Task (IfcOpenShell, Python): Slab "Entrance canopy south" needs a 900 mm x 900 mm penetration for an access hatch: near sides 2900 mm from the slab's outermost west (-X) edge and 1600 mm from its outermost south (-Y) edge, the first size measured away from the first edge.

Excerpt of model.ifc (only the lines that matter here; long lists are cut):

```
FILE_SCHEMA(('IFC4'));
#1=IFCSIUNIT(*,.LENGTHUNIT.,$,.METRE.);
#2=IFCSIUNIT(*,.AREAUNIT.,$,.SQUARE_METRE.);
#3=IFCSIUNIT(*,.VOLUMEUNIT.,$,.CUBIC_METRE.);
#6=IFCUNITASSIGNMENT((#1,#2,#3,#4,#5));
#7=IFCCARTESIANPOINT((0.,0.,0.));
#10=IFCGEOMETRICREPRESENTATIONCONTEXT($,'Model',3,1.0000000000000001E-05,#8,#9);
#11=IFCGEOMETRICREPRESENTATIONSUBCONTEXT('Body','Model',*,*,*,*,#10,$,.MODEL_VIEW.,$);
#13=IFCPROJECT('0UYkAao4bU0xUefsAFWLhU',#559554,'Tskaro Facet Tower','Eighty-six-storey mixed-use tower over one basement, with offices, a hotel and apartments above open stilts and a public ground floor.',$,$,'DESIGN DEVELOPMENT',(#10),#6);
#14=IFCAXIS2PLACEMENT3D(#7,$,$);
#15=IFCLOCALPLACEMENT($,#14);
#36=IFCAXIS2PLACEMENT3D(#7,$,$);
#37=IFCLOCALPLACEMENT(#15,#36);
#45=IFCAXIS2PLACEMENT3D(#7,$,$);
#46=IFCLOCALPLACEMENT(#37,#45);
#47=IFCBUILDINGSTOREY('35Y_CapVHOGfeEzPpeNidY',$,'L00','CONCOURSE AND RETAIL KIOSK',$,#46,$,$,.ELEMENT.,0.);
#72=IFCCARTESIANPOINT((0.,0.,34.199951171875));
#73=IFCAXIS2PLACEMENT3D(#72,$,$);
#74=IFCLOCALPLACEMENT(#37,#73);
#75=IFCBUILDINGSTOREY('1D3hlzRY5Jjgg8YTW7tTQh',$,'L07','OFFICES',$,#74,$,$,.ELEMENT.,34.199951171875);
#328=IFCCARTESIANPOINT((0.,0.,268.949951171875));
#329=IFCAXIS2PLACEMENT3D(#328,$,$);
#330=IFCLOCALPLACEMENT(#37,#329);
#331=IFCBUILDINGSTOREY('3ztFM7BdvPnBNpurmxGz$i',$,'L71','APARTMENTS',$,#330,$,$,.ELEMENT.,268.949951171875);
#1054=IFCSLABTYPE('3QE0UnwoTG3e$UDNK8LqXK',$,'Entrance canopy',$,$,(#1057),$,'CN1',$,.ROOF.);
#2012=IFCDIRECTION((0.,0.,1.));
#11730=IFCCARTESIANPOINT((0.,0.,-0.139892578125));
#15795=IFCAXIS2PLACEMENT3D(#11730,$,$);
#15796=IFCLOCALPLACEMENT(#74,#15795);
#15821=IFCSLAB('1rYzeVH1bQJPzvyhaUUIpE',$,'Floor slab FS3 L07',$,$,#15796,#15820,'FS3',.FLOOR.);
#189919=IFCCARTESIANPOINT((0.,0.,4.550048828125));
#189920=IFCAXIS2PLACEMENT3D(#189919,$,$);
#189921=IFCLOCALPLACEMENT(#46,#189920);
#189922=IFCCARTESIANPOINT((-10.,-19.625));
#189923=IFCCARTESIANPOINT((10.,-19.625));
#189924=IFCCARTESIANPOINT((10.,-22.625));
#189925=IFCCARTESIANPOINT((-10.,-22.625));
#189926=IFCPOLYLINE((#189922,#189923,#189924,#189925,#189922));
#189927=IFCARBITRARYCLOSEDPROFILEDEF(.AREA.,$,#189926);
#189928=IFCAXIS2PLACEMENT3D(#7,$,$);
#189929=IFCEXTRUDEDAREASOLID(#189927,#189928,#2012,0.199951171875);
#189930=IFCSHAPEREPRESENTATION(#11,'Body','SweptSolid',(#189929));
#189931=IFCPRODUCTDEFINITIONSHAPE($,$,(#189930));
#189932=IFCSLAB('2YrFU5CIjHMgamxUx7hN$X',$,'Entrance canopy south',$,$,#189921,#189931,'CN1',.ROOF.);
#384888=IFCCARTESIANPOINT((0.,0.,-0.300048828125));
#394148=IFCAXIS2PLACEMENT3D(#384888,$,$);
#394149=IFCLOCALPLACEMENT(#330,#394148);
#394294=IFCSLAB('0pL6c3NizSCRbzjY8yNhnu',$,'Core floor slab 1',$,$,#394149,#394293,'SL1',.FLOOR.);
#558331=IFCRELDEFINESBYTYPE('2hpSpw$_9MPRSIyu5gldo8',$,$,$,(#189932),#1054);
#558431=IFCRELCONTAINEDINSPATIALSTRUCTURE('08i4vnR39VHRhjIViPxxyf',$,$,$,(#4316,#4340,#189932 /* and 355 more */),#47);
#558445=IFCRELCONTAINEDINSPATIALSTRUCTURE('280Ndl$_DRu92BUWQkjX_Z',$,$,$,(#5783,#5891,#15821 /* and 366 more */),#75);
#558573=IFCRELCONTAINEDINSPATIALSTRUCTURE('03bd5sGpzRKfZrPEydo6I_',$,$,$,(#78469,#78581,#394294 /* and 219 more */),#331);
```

```python
import numpy as np
import ifcopenshell
import ifcopenshell.api.feature
import ifcopenshell.api.geometry
import ifcopenshell.api.root
import ifcopenshell.geom
import ifcopenshell.util.placement
import ifcopenshell.util.representation
import ifcopenshell.util.shape
import ifcopenshell.util.unit

model = ifcopenshell.open("model.ifc")
unit_scale = ifcopenshell.util.unit.calculate_unit_scale(model)
settings = ifcopenshell.geom.settings()


def volume(element):
    """Net volume in cubic metres, openings subtracted."""
    shape = ifcopenshell.geom.create_shape(settings, element)
    return ifcopenshell.util.shape.get_volume(shape.geometry)


slab = model.by_id(189932)
before = volume(slab)

# Extent in the slab's own axes, in metres. The edges named are its -X and -Y sides.
slab_shape = ifcopenshell.geom.create_shape(settings, slab)
vertices = ifcopenshell.util.shape.get_vertices(slab_shape.geometry)
x_min, y_min, bottom = vertices.min(axis=0)
top = vertices[:, 2].max()

opening = ifcopenshell.api.root.create_entity(model, ifc_class="IfcOpeningElement", name="Access hatch opening", predefined_type="OPENING")
context = ifcopenshell.util.representation.get_context(model, "Model", "Body", "MODEL_VIEW")
width, depth = 0.9, 0.9
outline = [(0.0, 0.0), (width, 0.0), (width, depth), (0.0, depth), (0.0, 0.0)]
# Overshoot both faces by 50 mm so the cut is clean.
shape = ifcopenshell.api.geometry.add_slab_representation(
    model, context=context, depth=top - bottom + 0.1, polyline=outline
)
ifcopenshell.api.geometry.assign_representation(model, product=opening, representation=shape)

matrix = ifcopenshell.util.placement.get_local_placement(slab.ObjectPlacement)
matrix[:, 3] = matrix @ np.append(np.array([x_min + 2.9, y_min + 1.6, bottom - 0.05]) / unit_scale, 1.0)
ifcopenshell.api.geometry.edit_object_placement(model, product=opening, matrix=matrix, is_si=False)
ifcopenshell.api.feature.add_feature(model, feature=opening, element=slab)

after = volume(slab)

print(f"slab volume {before:.3f} -> {after:.3f} m3")

model.write("model_rev.ifc")
```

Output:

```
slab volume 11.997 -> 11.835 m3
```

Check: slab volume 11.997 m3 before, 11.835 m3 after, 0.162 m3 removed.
